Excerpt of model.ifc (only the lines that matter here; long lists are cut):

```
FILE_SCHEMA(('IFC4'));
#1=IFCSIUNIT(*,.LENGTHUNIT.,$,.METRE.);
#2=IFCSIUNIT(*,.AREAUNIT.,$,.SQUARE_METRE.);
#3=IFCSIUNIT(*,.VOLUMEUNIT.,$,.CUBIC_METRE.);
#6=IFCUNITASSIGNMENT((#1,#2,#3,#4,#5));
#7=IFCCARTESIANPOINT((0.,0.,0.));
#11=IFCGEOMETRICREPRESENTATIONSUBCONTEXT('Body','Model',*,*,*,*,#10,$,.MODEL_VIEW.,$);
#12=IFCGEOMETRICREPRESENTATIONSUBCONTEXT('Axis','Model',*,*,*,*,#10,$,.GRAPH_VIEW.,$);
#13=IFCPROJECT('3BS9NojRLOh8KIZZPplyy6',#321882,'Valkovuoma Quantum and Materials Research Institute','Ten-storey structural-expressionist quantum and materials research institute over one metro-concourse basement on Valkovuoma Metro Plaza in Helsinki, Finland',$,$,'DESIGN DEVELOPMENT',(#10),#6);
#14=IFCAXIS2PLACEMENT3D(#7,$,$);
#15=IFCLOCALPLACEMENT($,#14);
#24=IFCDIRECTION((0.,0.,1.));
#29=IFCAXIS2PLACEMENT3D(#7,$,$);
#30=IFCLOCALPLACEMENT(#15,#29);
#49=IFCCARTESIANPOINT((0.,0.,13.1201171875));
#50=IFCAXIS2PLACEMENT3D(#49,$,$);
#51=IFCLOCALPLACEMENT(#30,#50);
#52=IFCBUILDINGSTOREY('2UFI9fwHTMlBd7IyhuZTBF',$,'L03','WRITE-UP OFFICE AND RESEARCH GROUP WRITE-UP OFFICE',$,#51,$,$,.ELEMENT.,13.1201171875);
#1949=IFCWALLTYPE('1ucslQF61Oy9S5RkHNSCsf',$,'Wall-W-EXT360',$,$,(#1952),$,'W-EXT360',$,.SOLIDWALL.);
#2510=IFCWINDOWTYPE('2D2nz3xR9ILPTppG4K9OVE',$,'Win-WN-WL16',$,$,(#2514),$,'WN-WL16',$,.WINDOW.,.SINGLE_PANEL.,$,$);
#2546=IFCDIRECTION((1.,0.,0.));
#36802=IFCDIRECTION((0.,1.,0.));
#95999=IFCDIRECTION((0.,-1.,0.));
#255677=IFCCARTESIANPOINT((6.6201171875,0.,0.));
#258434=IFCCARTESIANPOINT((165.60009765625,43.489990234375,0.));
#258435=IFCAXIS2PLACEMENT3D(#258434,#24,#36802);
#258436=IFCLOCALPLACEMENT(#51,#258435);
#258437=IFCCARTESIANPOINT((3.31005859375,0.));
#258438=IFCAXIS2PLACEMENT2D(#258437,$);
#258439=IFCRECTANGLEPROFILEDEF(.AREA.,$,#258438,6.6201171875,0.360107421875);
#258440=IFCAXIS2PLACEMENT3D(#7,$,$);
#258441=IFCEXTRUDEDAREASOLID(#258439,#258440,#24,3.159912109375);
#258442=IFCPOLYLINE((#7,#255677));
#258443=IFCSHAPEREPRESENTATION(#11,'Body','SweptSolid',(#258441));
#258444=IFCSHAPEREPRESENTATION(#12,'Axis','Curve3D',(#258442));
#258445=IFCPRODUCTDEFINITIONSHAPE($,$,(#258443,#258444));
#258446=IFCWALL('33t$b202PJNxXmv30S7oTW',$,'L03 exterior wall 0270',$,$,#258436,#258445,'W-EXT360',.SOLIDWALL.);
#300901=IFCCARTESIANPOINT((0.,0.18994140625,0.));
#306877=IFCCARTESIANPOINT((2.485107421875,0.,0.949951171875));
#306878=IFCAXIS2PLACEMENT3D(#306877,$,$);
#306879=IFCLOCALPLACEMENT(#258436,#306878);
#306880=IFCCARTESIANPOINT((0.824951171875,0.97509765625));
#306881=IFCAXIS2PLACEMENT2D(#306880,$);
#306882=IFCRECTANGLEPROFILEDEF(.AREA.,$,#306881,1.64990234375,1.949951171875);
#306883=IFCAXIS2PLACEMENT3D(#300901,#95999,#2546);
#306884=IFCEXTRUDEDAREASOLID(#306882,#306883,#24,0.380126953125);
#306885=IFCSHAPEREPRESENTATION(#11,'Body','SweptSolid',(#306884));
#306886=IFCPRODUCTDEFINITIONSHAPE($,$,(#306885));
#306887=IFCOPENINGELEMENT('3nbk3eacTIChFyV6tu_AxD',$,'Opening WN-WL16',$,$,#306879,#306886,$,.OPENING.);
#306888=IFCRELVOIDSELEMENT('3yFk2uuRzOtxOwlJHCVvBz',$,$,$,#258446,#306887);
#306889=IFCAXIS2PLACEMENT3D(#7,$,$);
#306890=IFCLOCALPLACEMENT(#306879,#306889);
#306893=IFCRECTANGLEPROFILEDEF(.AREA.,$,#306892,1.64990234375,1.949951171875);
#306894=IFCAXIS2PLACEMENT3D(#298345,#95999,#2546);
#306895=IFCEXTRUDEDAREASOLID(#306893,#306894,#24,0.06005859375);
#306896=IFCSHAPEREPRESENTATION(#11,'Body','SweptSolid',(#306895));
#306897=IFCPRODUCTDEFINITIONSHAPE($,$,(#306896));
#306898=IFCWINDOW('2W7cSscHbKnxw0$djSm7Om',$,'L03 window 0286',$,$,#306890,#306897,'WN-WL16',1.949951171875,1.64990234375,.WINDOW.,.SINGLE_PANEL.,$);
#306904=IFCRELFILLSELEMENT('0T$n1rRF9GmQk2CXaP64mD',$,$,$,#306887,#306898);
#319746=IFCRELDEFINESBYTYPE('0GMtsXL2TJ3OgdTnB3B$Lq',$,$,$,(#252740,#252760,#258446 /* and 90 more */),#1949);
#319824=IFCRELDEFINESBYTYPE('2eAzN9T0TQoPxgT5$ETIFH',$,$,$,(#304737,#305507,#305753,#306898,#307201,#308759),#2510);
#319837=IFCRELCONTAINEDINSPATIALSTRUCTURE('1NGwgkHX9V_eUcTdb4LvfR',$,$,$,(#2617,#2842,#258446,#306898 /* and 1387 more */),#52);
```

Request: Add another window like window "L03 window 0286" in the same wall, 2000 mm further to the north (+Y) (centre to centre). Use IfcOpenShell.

```python
import ifcopenshell
import ifcopenshell.api.feature
import ifcopenshell.api.geometry
import ifcopenshell.api.root
import ifcopenshell.geom
import ifcopenshell.util.element
import ifcopenshell.util.placement
import ifcopenshell.util.shape
import ifcopenshell.util.unit

model = ifcopenshell.open("model.ifc")
unit_scale = ifcopenshell.util.unit.calculate_unit_scale(model)
settings = ifcopenshell.geom.settings()


def volume(element):
    """Net volume in cubic metres, openings subtracted."""
    shape = ifcopenshell.geom.create_shape(settings, element)
    return ifcopenshell.util.shape.get_volume(shape.geometry)


window = model.by_guid("2W7cSscHbKnxw0$djSm7Om")
opening = window.FillsVoids[0].RelatingOpeningElement
wall = opening.VoidsElements[0].RelatingBuildingElement
before = volume(wall)
shift = ifcopenshell.util.placement.get_local_placement(wall.ObjectPlacement)[:3, 0] * 2 / unit_scale

# copy_class copies the void relationship, type, container and properties, but no geometry.
new_opening = ifcopenshell.api.root.copy_class(model, product=opening)
new_opening.Representation = ifcopenshell.util.element.copy_deep(
    model, opening.Representation, exclude=["IfcGeometricRepresentationContext", "IfcRepresentationMap"]
)
new_window = ifcopenshell.api.root.copy_class(model, product=window)
new_window.Representation = ifcopenshell.util.element.copy_deep(
    model, window.Representation, exclude=["IfcGeometricRepresentationContext", "IfcRepresentationMap"]
)
new_window.Tag = None
ifcopenshell.api.feature.add_filling(model, opening=new_opening, element=new_window)

for old, new in ((opening, new_opening), (window, new_window)):
    matrix = ifcopenshell.util.placement.get_local_placement(old.ObjectPlacement)
    matrix[:3, 3] += shift
    ifcopenshell.api.geometry.edit_object_placement(model, product=new, matrix=matrix, is_si=False)

after = volume(wall)

print(f"wall volume {before:.3f} -> {after:.3f} m3")

model.write("model_edited.ifc")
```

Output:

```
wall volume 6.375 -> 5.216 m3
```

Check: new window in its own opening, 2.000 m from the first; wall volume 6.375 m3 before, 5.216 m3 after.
